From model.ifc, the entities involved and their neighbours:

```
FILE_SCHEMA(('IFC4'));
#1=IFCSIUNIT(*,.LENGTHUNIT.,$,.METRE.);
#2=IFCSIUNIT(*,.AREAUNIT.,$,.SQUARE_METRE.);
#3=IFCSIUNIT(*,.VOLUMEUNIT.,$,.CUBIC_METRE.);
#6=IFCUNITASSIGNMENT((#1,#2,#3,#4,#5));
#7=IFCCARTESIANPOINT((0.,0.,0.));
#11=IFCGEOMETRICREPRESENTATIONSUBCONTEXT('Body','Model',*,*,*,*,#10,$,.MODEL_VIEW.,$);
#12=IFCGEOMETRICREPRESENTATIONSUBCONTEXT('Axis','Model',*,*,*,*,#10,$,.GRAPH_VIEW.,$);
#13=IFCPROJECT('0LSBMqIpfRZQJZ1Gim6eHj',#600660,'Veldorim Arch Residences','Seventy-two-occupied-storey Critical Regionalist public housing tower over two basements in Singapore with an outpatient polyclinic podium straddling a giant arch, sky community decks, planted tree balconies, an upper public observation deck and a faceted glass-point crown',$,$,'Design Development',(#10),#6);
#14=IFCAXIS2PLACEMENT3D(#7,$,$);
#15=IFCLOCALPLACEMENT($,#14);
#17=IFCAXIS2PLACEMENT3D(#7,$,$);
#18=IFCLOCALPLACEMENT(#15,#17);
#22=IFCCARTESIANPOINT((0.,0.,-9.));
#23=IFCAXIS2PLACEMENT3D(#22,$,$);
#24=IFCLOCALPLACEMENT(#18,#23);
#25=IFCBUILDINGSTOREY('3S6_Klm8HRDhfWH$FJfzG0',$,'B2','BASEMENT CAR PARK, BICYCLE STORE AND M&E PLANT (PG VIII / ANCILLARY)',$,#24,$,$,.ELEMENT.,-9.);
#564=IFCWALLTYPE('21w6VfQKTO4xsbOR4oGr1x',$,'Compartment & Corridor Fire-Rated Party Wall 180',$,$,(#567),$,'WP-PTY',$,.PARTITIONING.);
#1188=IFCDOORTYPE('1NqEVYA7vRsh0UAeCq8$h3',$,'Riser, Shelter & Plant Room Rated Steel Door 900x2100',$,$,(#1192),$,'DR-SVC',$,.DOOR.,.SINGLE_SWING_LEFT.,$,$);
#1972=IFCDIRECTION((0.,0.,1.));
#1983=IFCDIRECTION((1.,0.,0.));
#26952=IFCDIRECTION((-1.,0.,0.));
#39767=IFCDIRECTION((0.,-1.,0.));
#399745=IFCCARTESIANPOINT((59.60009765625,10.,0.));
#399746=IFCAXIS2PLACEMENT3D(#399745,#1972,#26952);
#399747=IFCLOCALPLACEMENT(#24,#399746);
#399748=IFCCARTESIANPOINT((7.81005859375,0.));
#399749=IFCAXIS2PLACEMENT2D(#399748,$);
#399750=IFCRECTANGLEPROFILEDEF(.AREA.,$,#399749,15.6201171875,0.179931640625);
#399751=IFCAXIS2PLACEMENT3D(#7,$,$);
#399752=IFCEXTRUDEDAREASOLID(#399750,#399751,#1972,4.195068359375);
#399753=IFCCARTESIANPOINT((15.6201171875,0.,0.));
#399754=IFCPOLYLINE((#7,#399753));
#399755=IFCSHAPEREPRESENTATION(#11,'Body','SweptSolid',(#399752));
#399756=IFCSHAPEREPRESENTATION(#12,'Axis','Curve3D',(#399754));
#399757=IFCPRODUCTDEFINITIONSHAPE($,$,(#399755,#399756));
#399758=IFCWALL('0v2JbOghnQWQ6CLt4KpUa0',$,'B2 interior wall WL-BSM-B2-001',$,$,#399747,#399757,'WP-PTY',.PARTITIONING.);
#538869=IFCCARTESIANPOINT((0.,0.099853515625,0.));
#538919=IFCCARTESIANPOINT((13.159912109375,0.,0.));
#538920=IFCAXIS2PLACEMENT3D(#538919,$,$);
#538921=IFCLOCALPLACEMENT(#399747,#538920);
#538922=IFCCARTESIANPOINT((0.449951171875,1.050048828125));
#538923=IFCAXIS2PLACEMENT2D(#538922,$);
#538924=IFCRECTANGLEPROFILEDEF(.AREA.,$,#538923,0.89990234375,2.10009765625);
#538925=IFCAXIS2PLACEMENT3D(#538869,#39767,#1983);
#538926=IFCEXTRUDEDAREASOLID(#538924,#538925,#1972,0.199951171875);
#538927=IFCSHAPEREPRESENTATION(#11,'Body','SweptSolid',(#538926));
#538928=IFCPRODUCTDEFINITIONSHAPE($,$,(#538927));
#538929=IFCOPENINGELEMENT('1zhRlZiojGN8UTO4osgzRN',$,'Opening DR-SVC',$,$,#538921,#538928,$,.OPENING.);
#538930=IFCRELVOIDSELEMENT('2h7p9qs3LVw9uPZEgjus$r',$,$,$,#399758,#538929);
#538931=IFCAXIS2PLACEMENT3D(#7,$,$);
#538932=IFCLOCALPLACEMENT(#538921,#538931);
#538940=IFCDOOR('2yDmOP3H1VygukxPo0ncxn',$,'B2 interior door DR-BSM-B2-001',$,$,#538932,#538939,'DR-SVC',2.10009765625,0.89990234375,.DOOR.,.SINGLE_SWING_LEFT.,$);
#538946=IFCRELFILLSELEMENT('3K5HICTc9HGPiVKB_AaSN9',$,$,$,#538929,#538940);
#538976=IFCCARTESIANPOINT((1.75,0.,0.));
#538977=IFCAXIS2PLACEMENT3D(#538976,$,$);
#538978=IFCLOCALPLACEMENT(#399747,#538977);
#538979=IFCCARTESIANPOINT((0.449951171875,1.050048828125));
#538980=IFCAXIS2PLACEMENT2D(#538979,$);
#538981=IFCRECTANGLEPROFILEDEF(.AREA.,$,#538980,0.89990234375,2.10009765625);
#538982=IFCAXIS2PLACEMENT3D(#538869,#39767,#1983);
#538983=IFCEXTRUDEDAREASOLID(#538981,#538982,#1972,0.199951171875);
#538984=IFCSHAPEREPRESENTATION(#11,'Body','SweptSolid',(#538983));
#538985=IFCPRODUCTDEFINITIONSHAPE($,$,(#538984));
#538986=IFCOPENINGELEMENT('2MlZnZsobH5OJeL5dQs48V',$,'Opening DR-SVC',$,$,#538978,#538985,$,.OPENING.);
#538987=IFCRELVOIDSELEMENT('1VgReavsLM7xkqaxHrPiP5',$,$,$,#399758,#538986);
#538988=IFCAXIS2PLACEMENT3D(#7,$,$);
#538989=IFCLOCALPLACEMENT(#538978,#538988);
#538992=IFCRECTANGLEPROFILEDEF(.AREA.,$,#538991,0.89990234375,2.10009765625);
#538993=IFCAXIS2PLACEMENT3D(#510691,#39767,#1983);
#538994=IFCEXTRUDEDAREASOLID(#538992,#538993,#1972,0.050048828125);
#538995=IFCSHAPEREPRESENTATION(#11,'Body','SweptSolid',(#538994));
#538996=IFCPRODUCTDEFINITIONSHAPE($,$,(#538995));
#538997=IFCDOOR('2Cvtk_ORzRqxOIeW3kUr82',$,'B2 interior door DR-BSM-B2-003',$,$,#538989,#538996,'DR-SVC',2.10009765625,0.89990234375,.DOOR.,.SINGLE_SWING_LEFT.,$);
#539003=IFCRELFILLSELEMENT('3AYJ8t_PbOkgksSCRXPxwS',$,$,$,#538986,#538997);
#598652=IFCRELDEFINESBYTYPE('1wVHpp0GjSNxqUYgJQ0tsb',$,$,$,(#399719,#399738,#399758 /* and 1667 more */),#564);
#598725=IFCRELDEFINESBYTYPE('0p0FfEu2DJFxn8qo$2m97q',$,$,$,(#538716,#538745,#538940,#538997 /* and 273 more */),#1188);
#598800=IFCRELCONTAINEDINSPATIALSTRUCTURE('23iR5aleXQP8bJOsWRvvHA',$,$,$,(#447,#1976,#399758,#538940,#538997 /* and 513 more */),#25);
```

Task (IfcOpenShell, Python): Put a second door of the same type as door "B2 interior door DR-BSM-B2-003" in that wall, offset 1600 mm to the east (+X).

```python
import ifcopenshell
import ifcopenshell.api.feature
import ifcopenshell.api.geometry
import ifcopenshell.api.root
import ifcopenshell.geom
import ifcopenshell.util.element
import ifcopenshell.util.placement
import ifcopenshell.util.shape
import ifcopenshell.util.unit

model = ifcopenshell.open("model.ifc")
unit_scale = ifcopenshell.util.unit.calculate_unit_scale(model)
settings = ifcopenshell.geom.settings()


def volume(element):
    """Net volume in cubic metres, openings subtracted."""
    shape = ifcopenshell.geom.create_shape(settings, element)
    return ifcopenshell.util.shape.get_volume(shape.geometry)


door = model.by_guid("2Cvtk_ORzRqxOIeW3kUr82")
opening = door.FillsVoids[0].RelatingOpeningElement
wall = opening.VoidsElements[0].RelatingBuildingElement
before = volume(wall)
shift = ifcopenshell.util.placement.get_local_placement(wall.ObjectPlacement)[:3, 0] * -1.6 / unit_scale

# copy_class copies the void relationship, type, container and properties, but no geometry.
new_opening = ifcopenshell.api.root.copy_class(model, product=opening)
new_opening.Representation = ifcopenshell.util.element.copy_deep(
    model, opening.Representation, exclude=["IfcGeometricRepresentationContext", "IfcRepresentationMap"]
)
new_door = ifcopenshell.api.root.copy_class(model, product=door)
new_door.Representation = ifcopenshell.util.element.copy_deep(
    model, door.Representation, exclude=["IfcGeometricRepresentationContext", "IfcRepresentationMap"]
)
new_door.Tag = None
ifcopenshell.api.feature.add_filling(model, opening=new_opening, element=new_door)

for old, new in ((opening, new_opening), (door, new_door)):
    matrix = ifcopenshell.util.placement.get_local_placement(old.ObjectPlacement)
    matrix[:3, 3] += shift
    ifcopenshell.api.geometry.edit_object_placement(model, product=new, matrix=matrix, is_si=False)

after = volume(wall)

print(f"wall volume {before:.3f} -> {after:.3f} m3")

model.write("model_edited.ifc")
```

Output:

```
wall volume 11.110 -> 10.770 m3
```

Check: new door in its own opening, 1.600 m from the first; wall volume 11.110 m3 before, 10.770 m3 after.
